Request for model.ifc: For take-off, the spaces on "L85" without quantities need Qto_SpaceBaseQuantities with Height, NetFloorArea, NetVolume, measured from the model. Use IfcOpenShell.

First a look at what the model holds.

```python
import ifcopenshell
import ifcopenshell.util.element
import ifcopenshell.util.unit

model = ifcopenshell.open("model.ifc")
print(model.schema)
for unit_type in ("LENGTHUNIT", "AREAUNIT", "VOLUMEUNIT"):
    print(unit_type, ifcopenshell.util.unit.calculate_unit_scale(model, unit_type))
storey = next(s for s in model.by_type("IfcBuildingStorey") if s.Name == "L85")
spaces = [e for e in ifcopenshell.util.element.get_decomposition(storey) if e.is_a("IfcSpace")]
for e in sorted(spaces, key=lambda e: e.id()):
    print(e.id(), e.is_a(), e.Name, list(ifcopenshell.util.element.get_psets(e, qtos_only=True)), sep=" | ")
```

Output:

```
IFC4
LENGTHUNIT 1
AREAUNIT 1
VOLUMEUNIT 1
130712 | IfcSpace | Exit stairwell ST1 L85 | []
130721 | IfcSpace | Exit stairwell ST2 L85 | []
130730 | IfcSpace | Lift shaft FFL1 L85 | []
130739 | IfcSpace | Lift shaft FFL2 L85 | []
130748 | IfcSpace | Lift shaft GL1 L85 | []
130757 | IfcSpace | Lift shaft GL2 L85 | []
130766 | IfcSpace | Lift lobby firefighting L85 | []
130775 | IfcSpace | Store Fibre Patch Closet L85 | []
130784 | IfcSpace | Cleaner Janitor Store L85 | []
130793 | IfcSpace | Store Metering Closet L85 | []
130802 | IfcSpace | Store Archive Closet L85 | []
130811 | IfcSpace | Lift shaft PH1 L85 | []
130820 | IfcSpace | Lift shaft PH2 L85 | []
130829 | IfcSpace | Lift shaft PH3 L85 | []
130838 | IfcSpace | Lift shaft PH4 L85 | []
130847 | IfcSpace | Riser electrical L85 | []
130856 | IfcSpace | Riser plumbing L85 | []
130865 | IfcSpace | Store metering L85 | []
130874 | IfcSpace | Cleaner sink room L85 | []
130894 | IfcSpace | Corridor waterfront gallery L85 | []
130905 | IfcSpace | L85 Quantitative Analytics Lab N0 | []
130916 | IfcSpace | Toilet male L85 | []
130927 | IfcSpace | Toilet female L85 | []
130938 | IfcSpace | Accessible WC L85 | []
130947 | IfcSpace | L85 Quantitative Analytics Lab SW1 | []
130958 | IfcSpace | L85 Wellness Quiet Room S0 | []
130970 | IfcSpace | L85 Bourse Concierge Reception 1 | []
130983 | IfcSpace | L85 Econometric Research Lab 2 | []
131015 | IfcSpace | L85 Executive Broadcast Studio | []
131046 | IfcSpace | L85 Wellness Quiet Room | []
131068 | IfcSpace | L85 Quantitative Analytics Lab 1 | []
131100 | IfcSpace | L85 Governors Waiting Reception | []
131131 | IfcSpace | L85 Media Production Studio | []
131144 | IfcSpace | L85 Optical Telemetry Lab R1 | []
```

```python
import ifcopenshell
import ifcopenshell.api.pset
import ifcopenshell.geom
import ifcopenshell.util.element
import ifcopenshell.util.shape
import ifcopenshell.util.unit

model = ifcopenshell.open("model.ifc")
unit_scale = ifcopenshell.util.unit.calculate_unit_scale(model)
area_scale = ifcopenshell.util.unit.calculate_unit_scale(model, "AREAUNIT")
volume_scale = ifcopenshell.util.unit.calculate_unit_scale(model, "VOLUMEUNIT")
settings = ifcopenshell.geom.settings()

storey = next(s for s in model.by_type("IfcBuildingStorey") if s.Name == "L85")
spaces = [e for e in ifcopenshell.util.element.get_decomposition(storey) if e.is_a("IfcSpace")]

for e in sorted(spaces, key=lambda e: e.id()):
    if ifcopenshell.util.element.get_psets(e, qtos_only=True, should_inherit=False):
        continue
    # Geometry comes back in metres, in the element's own axes.
    shape = ifcopenshell.geom.create_shape(settings, e)
    values = {
        "Height": ifcopenshell.util.shape.get_z(shape.geometry) / unit_scale,
        "NetFloorArea": ifcopenshell.util.shape.get_footprint_area(shape.geometry) / area_scale,
        "NetVolume": ifcopenshell.util.shape.get_volume(shape.geometry) / volume_scale,
    }
    qto = ifcopenshell.api.pset.add_qto(model, product=e, name="Qto_SpaceBaseQuantities")
    ifcopenshell.api.pset.edit_qto(model, qto=qto, properties=values)
    print(e.id(), {k: round(v, 3) for k, v in values.items()})

model.write("model_updated.ifc")
```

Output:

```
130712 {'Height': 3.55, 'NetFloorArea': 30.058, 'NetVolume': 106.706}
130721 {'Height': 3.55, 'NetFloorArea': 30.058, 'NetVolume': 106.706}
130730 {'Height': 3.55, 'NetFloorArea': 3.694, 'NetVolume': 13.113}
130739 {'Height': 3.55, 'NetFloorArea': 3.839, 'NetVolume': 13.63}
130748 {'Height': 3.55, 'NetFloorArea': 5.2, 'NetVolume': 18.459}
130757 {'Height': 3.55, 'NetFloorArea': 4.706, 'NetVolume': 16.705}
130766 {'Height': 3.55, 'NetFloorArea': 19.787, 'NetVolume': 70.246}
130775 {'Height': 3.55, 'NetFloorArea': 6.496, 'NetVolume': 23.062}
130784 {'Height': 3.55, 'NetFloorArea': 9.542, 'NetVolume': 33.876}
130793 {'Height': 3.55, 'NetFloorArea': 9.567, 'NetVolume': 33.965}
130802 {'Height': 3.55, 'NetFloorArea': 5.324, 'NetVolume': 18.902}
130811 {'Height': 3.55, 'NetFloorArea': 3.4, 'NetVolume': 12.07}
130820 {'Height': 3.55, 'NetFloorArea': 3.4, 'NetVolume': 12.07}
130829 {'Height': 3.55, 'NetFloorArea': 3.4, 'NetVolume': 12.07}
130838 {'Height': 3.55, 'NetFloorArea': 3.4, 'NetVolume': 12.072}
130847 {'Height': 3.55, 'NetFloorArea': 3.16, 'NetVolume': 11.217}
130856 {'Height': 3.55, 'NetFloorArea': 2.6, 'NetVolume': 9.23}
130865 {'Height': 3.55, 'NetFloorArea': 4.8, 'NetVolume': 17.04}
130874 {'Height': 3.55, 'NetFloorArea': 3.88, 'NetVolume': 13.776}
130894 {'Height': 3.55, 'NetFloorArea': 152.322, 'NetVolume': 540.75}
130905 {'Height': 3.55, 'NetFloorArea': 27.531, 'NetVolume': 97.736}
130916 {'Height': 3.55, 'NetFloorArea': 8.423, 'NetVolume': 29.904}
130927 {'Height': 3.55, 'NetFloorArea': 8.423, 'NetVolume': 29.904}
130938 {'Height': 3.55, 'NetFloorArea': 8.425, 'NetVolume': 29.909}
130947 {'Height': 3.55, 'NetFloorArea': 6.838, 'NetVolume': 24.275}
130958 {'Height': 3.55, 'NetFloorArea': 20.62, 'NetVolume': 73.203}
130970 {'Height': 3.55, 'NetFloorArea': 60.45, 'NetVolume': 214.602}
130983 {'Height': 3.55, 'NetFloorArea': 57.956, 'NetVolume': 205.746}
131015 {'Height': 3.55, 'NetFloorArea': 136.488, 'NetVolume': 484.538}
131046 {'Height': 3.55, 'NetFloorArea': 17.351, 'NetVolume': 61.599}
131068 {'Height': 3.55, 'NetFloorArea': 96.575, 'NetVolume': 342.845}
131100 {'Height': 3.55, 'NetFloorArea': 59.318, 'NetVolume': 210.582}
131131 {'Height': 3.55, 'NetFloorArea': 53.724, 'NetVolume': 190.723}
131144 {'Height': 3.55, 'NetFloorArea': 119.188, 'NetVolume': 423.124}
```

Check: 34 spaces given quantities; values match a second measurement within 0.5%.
